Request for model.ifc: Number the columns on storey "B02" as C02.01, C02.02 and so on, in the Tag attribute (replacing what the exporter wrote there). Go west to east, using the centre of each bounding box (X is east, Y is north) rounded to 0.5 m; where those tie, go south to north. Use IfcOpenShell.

First a look at what the model holds.

```python
import ifcopenshell
import ifcopenshell.util.element
import ifcopenshell.util.placement

model = ifcopenshell.open("model.ifc")
print(model.schema)
storey = next(s for s in model.by_type("IfcBuildingStorey") if s.Name == "B02")
columns = [e for e in ifcopenshell.util.element.get_decomposition(storey) if e.is_a("IfcColumn")]
for e in sorted(columns, key=lambda e: e.id()):
    origin = ifcopenshell.util.placement.get_local_placement(e.ObjectPlacement)[:3, 3]
    print(e.id(), e.Tag, e.Name, origin.round(2) + 0.0, sep=" | ")
```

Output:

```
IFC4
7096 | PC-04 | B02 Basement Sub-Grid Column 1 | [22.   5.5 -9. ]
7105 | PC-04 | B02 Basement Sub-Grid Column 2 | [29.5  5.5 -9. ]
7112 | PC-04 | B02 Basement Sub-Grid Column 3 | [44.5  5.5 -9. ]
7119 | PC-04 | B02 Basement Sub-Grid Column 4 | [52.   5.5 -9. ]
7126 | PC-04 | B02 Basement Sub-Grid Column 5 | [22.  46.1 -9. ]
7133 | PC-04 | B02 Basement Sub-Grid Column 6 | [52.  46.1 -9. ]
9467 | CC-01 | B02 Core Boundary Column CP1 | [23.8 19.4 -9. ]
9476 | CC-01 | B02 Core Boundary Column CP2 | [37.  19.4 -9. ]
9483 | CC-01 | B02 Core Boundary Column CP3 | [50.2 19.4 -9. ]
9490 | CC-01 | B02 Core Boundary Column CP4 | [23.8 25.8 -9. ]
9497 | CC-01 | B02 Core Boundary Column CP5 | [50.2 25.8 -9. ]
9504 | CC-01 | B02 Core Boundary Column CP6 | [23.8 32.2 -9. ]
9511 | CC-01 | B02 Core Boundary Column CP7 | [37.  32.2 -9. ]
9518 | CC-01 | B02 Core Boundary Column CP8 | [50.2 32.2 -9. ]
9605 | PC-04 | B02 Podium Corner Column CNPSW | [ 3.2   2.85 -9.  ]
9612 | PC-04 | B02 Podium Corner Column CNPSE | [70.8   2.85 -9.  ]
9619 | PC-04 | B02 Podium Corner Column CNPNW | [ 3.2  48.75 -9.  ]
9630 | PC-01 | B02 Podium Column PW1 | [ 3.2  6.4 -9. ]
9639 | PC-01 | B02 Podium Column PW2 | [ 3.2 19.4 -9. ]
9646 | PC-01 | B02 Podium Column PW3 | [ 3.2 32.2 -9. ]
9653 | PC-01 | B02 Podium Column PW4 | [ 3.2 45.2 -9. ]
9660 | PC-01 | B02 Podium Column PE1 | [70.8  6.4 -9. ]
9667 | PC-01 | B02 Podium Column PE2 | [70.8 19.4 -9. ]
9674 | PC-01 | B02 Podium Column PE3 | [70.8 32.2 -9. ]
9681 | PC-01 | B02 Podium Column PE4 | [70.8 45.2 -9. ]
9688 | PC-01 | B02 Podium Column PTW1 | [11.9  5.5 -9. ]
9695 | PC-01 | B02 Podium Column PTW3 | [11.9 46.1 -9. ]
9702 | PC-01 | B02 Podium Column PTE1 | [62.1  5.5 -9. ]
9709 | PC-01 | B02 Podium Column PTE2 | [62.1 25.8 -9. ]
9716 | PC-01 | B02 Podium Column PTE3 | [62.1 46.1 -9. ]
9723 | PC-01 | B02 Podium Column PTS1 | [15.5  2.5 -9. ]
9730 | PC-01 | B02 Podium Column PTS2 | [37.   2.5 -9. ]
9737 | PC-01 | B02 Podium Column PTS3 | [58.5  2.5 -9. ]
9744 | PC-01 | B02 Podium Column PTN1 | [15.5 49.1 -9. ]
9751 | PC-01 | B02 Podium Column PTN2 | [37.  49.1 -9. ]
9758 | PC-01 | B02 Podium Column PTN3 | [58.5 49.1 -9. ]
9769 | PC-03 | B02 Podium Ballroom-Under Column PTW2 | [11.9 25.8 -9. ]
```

```python
import ifcopenshell
import ifcopenshell.geom
import ifcopenshell.util.element
import ifcopenshell.util.shape

model = ifcopenshell.open("model.ifc")
settings = ifcopenshell.geom.settings()
settings.set("use-world-coords", True)


def centre(element):
    shape = ifcopenshell.geom.create_shape(settings, element)
    return ifcopenshell.util.shape.get_bbox_centroid(shape.geometry)


storey = next(s for s in model.by_type("IfcBuildingStorey") if s.Name == "B02")
columns = [e for e in ifcopenshell.util.element.get_decomposition(storey) if e.is_a("IfcColumn")]

# Insertion points can sit at a corner or the storey origin, so sort by the geometry (in metres).
centres = {e: centre(e) for e in columns}
columns.sort(key=lambda e: (round(centres[e][0] / 0.5), centres[e][1]))

for i, e in enumerate(columns, start=1):
    number = f"C02.{i:02d}"
    e.Tag = number
    print(e.id(), number)

model.write("model-out.ifc")
```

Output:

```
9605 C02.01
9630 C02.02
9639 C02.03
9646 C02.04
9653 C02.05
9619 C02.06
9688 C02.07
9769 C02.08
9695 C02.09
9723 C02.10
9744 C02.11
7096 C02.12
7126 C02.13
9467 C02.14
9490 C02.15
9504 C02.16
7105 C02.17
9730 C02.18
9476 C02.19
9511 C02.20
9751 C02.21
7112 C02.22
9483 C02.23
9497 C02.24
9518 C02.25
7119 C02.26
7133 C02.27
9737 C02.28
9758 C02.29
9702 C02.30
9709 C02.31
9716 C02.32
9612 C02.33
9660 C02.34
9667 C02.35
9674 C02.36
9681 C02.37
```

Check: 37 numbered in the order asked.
